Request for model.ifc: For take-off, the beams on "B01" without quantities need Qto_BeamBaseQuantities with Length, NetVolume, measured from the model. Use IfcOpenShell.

First a look at what the model holds.

```python
import ifcopenshell
import ifcopenshell.util.element
import ifcopenshell.util.unit

model = ifcopenshell.open("model.ifc")
print(model.schema)
for unit_type in ("LENGTHUNIT", "AREAUNIT", "VOLUMEUNIT"):
    print(unit_type, ifcopenshell.util.unit.calculate_unit_scale(model, unit_type))
storey = next(s for s in model.by_type("IfcBuildingStorey") if s.Name == "B01")
beams = [e for e in ifcopenshell.util.element.get_decomposition(storey) if e.is_a("IfcBeam")]
for e in sorted(beams, key=lambda e: e.id()):
    print(e.id(), e.is_a(), e.Name, list(ifcopenshell.util.element.get_psets(e, qtos_only=True)), sep=" | ")
```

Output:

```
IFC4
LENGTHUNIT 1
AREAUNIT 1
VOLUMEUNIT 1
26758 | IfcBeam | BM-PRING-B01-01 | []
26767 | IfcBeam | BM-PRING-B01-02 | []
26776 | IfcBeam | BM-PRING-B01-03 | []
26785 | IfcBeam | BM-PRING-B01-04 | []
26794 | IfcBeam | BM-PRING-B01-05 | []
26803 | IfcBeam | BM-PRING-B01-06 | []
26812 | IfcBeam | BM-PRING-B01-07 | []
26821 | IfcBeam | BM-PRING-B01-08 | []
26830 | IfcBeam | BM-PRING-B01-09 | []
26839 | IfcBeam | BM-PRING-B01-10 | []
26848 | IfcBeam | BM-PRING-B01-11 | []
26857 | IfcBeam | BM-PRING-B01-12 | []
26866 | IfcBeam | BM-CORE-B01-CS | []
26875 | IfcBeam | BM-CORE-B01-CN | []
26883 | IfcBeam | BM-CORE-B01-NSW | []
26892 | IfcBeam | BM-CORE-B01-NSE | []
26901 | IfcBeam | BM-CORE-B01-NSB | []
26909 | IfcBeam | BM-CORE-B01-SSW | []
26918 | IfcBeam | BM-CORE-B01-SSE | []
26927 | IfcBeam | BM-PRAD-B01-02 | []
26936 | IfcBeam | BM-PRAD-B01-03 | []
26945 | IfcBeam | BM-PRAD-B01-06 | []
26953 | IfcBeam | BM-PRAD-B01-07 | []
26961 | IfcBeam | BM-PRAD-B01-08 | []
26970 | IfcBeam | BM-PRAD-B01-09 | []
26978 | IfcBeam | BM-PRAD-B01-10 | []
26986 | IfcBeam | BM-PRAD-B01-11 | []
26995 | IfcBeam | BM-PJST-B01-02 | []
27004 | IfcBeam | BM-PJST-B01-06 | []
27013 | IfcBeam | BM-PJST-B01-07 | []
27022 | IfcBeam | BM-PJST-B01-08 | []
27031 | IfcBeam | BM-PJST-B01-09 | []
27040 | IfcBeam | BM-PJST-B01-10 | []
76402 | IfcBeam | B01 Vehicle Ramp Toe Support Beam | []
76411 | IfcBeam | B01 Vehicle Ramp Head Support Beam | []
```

```python
import ifcopenshell
import ifcopenshell.api.pset
import ifcopenshell.geom
import ifcopenshell.util.element
import ifcopenshell.util.shape
import ifcopenshell.util.unit

model = ifcopenshell.open("model.ifc")
unit_scale = ifcopenshell.util.unit.calculate_unit_scale(model)
volume_scale = ifcopenshell.util.unit.calculate_unit_scale(model, "VOLUMEUNIT")
settings = ifcopenshell.geom.settings()

storey = next(s for s in model.by_type("IfcBuildingStorey") if s.Name == "B01")
beams = [e for e in ifcopenshell.util.element.get_decomposition(storey) if e.is_a("IfcBeam")]

for e in sorted(beams, key=lambda e: e.id()):
    if ifcopenshell.util.element.get_psets(e, qtos_only=True, should_inherit=False):
        continue
    # Geometry comes back in metres, in the element's own axes.
    shape = ifcopenshell.geom.create_shape(settings, e)
    values = {
        "Length": ifcopenshell.util.shape.get_max_xyz(shape.geometry) / unit_scale,
        "NetVolume": ifcopenshell.util.shape.get_volume(shape.geometry) / volume_scale,
    }
    qto = ifcopenshell.api.pset.add_qto(model, product=e, name="Qto_BeamBaseQuantities")
    ifcopenshell.api.pset.edit_qto(model, qto=qto, properties=values)
    print(e.id(), {k: round(v, 3) for k, v in values.items()})

model.write("model_updated.ifc")
```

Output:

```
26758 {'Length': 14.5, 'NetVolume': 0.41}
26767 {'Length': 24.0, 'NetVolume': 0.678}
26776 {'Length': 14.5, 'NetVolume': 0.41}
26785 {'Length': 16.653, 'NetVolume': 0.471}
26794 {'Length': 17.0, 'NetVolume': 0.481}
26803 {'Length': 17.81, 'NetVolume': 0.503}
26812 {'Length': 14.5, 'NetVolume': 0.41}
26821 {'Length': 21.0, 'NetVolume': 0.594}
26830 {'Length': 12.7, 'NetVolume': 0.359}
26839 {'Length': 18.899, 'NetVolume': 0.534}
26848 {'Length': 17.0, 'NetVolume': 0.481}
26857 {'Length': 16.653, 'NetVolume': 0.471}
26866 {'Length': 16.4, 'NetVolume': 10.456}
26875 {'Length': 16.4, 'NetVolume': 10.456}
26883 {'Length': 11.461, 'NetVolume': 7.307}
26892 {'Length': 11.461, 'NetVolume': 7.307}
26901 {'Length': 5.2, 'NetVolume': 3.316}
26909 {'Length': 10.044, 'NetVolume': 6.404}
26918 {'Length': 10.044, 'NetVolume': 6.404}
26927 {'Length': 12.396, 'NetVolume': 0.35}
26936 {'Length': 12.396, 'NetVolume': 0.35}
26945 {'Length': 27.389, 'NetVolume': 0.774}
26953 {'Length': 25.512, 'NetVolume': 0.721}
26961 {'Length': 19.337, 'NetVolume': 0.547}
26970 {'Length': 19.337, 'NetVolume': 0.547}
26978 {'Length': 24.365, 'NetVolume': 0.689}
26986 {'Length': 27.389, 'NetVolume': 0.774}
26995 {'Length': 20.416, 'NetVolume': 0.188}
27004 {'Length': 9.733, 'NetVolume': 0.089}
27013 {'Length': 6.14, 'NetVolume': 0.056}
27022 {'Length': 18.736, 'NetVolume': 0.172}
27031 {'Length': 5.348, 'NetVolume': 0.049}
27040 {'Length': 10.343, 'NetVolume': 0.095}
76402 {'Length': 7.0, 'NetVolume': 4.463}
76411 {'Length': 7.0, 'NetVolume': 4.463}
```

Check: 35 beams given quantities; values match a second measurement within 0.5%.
